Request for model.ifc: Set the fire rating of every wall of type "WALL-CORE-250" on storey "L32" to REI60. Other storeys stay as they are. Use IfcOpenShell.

First a look at what the model holds.

```python
import ifcopenshell
import ifcopenshell.util.element

model = ifcopenshell.open("model.ifc")
print(model.schema)
storey = next(s for s in model.by_type("IfcBuildingStorey") if s.Name == "L32")
walls = [e for e in ifcopenshell.util.element.get_decomposition(storey) if e.is_a("IfcWall")]
seen = {}
for e in walls:
    element_type = ifcopenshell.util.element.get_type(e)
    key = (element_type.Name if element_type != e and element_type else None, ifcopenshell.util.element.get_pset(e, "Pset_WallCommon", "FireRating"))
    seen[key] = seen.get(key, 0) + 1
for (name, value), count in sorted(seen.items(), key=str):
    print(count, "x", name, "|", value)
```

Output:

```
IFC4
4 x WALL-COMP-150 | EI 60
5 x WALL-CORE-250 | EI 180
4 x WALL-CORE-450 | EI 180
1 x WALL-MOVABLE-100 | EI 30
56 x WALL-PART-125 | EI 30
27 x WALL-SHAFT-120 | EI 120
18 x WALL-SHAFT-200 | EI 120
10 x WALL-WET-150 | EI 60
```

```python
import ifcopenshell
import ifcopenshell.api.pset
import ifcopenshell.util.element

model = ifcopenshell.open("model.ifc")

storey = next(s for s in model.by_type("IfcBuildingStorey") if s.Name == "L32")
walls = [e for e in ifcopenshell.util.element.get_decomposition(storey) if e.is_a("IfcWall")]

count = 0
for e in walls:
    element_type = ifcopenshell.util.element.get_type(e)
    if element_type in (None, e) or element_type.Name != "WALL-CORE-250":
        continue
    # add_pset returns the element's existing set when there is one.
    pset = ifcopenshell.api.pset.add_pset(model, product=e, name="Pset_WallCommon")
    ifcopenshell.api.pset.edit_pset(model, pset=pset, properties={"FireRating": "REI60"})
    count += 1

print(count, "walls updated")

model.write("model_edited.ifc")
```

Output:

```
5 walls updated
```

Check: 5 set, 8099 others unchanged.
